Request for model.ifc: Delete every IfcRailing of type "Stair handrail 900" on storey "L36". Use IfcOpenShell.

First a look at what the model holds.

```python
import ifcopenshell
import ifcopenshell.util.element

model = ifcopenshell.open("model.ifc")
print(model.schema)
storey = next(s for s in model.by_type("IfcBuildingStorey") if s.Name == "L36")
railings = [e for e in ifcopenshell.util.element.get_decomposition(storey) if e.is_a("IfcRailing")]
seen = {}
for e in railings:
    element_type = ifcopenshell.util.element.get_type(e)
    name = element_type.Name if element_type not in (None, e) else None
    seen[name] = seen.get(name, 0) + 1
for name, count in sorted(seen.items(), key=str):
    print(count, "x", name)
```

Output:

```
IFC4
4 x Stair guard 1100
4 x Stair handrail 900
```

```python
import ifcopenshell
import ifcopenshell.api.root
import ifcopenshell.util.element

model = ifcopenshell.open("model.ifc")

storey = next(s for s in model.by_type("IfcBuildingStorey") if s.Name == "L36")
railings = [e for e in ifcopenshell.util.element.get_decomposition(storey) if e.is_a("IfcRailing")]
targets = [e for e in railings if (t := ifcopenshell.util.element.get_type(e)) not in (None, e) and t.Name == "Stair handrail 900"]

for e in targets:
    ifcopenshell.api.root.remove_product(model, product=e)
print(len(targets), "removed")

model.write("model_rev.ifc")
```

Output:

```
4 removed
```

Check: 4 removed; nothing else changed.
